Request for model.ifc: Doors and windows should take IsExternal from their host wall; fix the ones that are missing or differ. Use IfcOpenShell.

First a look at what the model holds.

```python
import ifcopenshell
import ifcopenshell.util.element

model = ifcopenshell.open("model.ifc")
print(model.schema)
seen = {}
for e in model.by_type("IfcDoor") + model.by_type("IfcWindow"):
    if not e.FillsVoids:
        continue
    host = e.FillsVoids[0].RelatingOpeningElement.VoidsElements[0].RelatingBuildingElement
    own = ifcopenshell.util.element.get_pset(e, f"Pset_{e.is_a()[3:].removesuffix('StandardCase')}Common", "IsExternal")
    wall = ifcopenshell.util.element.get_pset(host, "Pset_WallCommon", "IsExternal")
    seen[e.is_a(), own, wall] = seen.get((e.is_a(), own, wall), 0) + 1
for (cls, own, wall), count in sorted(seen.items(), key=str):
    print(count, cls, "IsExternal:", own, "| host wall:", wall)
```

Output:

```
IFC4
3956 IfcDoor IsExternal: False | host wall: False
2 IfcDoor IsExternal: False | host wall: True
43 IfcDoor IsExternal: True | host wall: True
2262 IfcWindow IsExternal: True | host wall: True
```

```python
import ifcopenshell
import ifcopenshell.api.pset
import ifcopenshell.util.element

model = ifcopenshell.open("model.ifc")

count = 0
for ifc_class, pset_name in (("IfcDoor", "Pset_DoorCommon"), ("IfcWindow", "Pset_WindowCommon")):
    for e in model.by_type(ifc_class):
        if not e.FillsVoids:
            continue
        host = e.FillsVoids[0].RelatingOpeningElement.VoidsElements[0].RelatingBuildingElement
        external = ifcopenshell.util.element.get_pset(host, "Pset_WallCommon", "IsExternal")
        if external is None or ifcopenshell.util.element.get_pset(e, pset_name, "IsExternal") == external:
            continue
        found = ifcopenshell.util.element.get_pset(e, pset_name, should_inherit=False)
        if found:
            pset = model.by_id(found["id"])
            if len(ifcopenshell.util.element.get_elements_by_pset(pset)) > 1:
                pset = ifcopenshell.api.pset.unshare_pset(model, products=[e], pset=pset)[0]
        else:
            pset = ifcopenshell.api.pset.add_pset(model, product=e, name=pset_name)
        ifcopenshell.api.pset.edit_pset(model, pset=pset, properties={"IsExternal": external})
        count += 1

print(count, "updated")

model.write("model_edited.ifc")
```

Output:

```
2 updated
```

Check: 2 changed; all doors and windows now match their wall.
